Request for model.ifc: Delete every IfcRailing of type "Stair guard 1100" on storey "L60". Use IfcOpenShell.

First a look at what the model holds.

```python
import ifcopenshell
import ifcopenshell.util.element

model = ifcopenshell.open("model.ifc")
print(model.schema)
storey = next(s for s in model.by_type("IfcBuildingStorey") if s.Name == "L60")
railings = [e for e in ifcopenshell.util.element.get_decomposition(storey) if e.is_a("IfcRailing")]
seen = {}
for e in railings:
    element_type = ifcopenshell.util.element.get_type(e)
    name = element_type.Name if element_type not in (None, e) else None
    seen[name] = seen.get(name, 0) + 1
for name, count in sorted(seen.items(), key=str):
    print(count, "x", name)
```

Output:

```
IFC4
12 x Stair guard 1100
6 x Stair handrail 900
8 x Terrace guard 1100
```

```python
import ifcopenshell
import ifcopenshell.api.root
import ifcopenshell.util.element

model = ifcopenshell.open("model.ifc")

storey = next(s for s in model.by_type("IfcBuildingStorey") if s.Name == "L60")
railings = [e for e in ifcopenshell.util.element.get_decomposition(storey) if e.is_a("IfcRailing")]
targets = [e for e in railings if (t := ifcopenshell.util.element.get_type(e)) not in (None, e) and t.Name == "Stair guard 1100"]

for e in targets:
    ifcopenshell.api.root.remove_product(model, product=e)
print(len(targets), "removed")

model.write("model_edited.ifc")
```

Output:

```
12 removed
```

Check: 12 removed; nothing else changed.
